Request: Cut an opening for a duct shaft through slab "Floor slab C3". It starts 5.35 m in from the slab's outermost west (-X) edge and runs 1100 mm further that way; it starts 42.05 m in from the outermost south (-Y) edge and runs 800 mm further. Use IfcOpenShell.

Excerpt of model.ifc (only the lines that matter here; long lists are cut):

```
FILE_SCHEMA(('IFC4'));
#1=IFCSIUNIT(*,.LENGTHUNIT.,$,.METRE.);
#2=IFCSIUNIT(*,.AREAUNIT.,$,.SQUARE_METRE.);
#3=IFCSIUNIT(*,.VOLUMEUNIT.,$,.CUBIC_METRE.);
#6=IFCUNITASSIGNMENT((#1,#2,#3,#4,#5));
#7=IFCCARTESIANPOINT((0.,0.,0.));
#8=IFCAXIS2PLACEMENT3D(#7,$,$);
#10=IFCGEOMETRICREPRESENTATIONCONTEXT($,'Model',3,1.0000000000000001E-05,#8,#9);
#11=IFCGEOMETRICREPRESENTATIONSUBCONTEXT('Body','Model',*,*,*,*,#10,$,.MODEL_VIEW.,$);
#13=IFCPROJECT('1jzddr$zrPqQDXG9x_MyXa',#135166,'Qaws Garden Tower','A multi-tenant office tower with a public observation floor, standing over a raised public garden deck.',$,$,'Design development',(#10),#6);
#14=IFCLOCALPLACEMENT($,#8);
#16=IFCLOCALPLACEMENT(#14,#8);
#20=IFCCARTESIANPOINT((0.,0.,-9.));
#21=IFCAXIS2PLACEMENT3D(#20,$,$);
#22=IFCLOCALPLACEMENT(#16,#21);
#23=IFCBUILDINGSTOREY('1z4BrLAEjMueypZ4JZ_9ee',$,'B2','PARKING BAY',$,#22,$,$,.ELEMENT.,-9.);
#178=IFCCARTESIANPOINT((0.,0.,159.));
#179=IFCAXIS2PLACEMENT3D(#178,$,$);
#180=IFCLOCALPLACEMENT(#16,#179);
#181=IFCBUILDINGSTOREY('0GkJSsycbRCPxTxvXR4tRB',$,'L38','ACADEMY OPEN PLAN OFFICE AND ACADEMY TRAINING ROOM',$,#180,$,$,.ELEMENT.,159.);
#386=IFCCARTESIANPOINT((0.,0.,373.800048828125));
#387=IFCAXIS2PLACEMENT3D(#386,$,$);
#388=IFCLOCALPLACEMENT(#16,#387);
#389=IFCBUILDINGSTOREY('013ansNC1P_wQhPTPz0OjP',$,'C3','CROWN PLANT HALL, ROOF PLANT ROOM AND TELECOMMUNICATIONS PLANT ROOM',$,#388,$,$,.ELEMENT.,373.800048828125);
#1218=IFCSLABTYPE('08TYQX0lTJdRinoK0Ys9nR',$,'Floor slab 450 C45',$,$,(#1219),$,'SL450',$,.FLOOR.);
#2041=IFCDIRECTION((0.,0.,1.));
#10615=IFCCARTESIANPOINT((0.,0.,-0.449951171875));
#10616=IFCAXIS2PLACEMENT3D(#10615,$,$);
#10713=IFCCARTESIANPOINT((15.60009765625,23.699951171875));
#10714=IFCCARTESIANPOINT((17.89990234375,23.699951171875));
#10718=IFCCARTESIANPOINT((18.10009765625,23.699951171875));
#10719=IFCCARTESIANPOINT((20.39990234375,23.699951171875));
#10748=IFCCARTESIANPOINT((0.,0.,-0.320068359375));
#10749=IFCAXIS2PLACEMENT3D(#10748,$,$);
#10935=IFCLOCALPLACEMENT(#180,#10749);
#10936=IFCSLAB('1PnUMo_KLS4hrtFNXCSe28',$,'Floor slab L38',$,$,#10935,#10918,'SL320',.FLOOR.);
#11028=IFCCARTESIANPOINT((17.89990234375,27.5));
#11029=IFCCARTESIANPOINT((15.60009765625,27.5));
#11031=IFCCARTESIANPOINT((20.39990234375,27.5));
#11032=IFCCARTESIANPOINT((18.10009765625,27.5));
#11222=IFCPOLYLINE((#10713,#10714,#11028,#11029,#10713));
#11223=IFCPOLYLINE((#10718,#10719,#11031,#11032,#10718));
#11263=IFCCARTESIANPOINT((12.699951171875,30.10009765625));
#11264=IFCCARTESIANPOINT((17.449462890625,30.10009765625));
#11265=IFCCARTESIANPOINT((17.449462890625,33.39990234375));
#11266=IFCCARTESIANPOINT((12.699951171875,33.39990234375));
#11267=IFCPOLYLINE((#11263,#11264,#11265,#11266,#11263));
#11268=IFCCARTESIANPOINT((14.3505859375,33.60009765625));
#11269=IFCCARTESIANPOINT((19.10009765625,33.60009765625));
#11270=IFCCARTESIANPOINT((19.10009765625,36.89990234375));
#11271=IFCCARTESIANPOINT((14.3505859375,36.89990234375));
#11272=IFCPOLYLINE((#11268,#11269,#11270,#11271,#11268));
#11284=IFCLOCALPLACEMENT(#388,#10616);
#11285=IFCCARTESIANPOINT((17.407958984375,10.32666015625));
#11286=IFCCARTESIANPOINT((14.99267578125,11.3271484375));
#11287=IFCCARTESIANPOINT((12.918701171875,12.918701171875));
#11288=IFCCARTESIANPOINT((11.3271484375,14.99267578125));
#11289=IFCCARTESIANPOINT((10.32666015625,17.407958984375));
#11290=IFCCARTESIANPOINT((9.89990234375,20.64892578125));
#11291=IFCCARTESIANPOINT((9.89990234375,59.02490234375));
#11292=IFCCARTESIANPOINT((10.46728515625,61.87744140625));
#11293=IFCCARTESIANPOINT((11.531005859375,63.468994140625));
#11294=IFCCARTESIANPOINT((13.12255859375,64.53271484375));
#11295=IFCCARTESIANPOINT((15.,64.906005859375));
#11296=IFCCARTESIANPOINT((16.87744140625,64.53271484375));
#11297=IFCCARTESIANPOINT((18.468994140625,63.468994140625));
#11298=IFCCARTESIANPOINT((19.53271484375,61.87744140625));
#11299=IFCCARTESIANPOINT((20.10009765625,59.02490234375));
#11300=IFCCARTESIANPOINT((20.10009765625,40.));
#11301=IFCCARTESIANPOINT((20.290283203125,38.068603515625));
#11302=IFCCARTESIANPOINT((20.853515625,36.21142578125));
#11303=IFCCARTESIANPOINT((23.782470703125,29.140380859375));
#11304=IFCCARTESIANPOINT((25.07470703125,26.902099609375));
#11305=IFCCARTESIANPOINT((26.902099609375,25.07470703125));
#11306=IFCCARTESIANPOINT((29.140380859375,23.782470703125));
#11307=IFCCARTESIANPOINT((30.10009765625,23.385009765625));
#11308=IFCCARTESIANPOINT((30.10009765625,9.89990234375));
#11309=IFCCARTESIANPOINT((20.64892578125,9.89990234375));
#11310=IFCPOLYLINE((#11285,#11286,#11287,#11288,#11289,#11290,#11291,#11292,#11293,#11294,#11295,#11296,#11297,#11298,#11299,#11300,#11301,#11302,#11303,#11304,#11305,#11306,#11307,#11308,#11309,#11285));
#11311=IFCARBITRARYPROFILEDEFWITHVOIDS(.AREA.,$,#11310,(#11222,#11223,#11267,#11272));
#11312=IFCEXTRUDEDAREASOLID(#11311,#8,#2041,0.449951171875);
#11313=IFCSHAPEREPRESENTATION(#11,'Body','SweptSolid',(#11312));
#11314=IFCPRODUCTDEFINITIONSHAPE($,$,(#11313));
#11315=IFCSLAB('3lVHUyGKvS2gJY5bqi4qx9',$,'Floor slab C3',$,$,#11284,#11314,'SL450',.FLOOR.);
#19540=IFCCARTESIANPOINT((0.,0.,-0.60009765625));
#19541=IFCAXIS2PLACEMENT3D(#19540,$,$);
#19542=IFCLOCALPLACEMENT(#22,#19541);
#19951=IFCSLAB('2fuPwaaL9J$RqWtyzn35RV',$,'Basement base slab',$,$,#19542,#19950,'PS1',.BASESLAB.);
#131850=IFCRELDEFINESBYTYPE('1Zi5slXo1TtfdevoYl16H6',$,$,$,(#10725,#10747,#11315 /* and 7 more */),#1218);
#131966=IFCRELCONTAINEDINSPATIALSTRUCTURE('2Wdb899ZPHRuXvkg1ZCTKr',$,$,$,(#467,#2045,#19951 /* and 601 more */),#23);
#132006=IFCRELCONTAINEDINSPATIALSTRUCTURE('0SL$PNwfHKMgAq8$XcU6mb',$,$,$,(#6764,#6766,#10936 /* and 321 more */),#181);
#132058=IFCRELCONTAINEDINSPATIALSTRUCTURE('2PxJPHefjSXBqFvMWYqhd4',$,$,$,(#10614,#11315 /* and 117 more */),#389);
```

```python
import numpy as np
import ifcopenshell
import ifcopenshell.api.feature
import ifcopenshell.api.geometry
import ifcopenshell.api.root
import ifcopenshell.geom
import ifcopenshell.util.placement
import ifcopenshell.util.representation
import ifcopenshell.util.shape
import ifcopenshell.util.unit

model = ifcopenshell.open("model.ifc")
unit_scale = ifcopenshell.util.unit.calculate_unit_scale(model)
settings = ifcopenshell.geom.settings()


def volume(element):
    """Net volume in cubic metres, openings subtracted."""
    shape = ifcopenshell.geom.create_shape(settings, element)
    return ifcopenshell.util.shape.get_volume(shape.geometry)


slab = model.by_guid("3lVHUyGKvS2gJY5bqi4qx9")
before = volume(slab)

# Extent in the slab's own axes, in metres. The edges named are its -X and -Y sides.
slab_shape = ifcopenshell.geom.create_shape(settings, slab)
vertices = ifcopenshell.util.shape.get_vertices(slab_shape.geometry)
x_min, y_min, bottom = vertices.min(axis=0)
top = vertices[:, 2].max()

opening = ifcopenshell.api.root.create_entity(model, ifc_class="IfcOpeningElement", name="Duct shaft opening", predefined_type="OPENING")
context = ifcopenshell.util.representation.get_context(model, "Model", "Body", "MODEL_VIEW")
width, depth = 1.1, 0.8
outline = [(0.0, 0.0), (width, 0.0), (width, depth), (0.0, depth), (0.0, 0.0)]
# Overshoot both faces by 50 mm so the cut is clean.
shape = ifcopenshell.api.geometry.add_slab_representation(
    model, context=context, depth=top - bottom + 0.1, polyline=outline
)
ifcopenshell.api.geometry.assign_representation(model, product=opening, representation=shape)

matrix = ifcopenshell.util.placement.get_local_placement(slab.ObjectPlacement)
matrix[:, 3] = matrix @ np.append(np.array([x_min + 5.35, y_min + 42.05, bottom - 0.05]) / unit_scale, 1.0)
ifcopenshell.api.geometry.edit_object_placement(model, product=opening, matrix=matrix, is_si=False)
ifcopenshell.api.feature.add_feature(model, feature=opening, element=slab)

after = volume(slab)

print(f"slab volume {before:.3f} -> {after:.3f} m3")

model.write("model_edited.ifc")
```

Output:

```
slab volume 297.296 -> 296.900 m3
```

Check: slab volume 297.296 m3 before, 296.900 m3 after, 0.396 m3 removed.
